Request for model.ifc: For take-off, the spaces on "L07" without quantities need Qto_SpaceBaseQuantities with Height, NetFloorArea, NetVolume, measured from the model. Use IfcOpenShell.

First a look at what the model holds.

```python
import ifcopenshell
import ifcopenshell.util.element
import ifcopenshell.util.unit

model = ifcopenshell.open("model.ifc")
print(model.schema)
for unit_type in ("LENGTHUNIT", "AREAUNIT", "VOLUMEUNIT"):
    print(unit_type, ifcopenshell.util.unit.calculate_unit_scale(model, unit_type))
storey = next(s for s in model.by_type("IfcBuildingStorey") if s.Name == "L07")
spaces = [e for e in ifcopenshell.util.element.get_decomposition(storey) if e.is_a("IfcSpace")]
for e in sorted(spaces, key=lambda e: e.id()):
    print(e.id(), e.is_a(), e.Name, list(ifcopenshell.util.element.get_psets(e, qtos_only=True)), sep=" | ")
```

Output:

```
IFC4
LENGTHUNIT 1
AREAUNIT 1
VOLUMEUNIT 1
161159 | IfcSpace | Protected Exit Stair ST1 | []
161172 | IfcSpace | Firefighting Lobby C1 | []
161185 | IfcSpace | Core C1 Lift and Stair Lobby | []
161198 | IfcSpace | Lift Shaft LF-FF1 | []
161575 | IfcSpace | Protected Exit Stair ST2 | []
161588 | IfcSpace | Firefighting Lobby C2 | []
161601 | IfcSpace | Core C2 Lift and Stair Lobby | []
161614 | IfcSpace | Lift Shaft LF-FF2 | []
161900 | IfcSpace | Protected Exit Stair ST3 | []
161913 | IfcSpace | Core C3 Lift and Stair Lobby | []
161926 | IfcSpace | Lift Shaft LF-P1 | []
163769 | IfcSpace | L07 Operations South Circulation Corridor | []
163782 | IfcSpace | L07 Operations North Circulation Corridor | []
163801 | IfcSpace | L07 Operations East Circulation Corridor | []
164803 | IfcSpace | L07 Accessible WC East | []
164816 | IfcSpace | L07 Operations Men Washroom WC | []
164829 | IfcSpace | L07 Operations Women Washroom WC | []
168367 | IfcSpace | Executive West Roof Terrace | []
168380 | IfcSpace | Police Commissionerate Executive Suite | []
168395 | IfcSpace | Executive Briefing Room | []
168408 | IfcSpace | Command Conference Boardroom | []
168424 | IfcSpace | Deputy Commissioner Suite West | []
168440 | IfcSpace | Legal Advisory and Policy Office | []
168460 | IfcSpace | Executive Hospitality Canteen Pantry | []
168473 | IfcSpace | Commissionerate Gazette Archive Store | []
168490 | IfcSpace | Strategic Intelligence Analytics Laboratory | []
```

```python
import ifcopenshell
import ifcopenshell.api.pset
import ifcopenshell.geom
import ifcopenshell.util.element
import ifcopenshell.util.shape
import ifcopenshell.util.unit

model = ifcopenshell.open("model.ifc")
unit_scale = ifcopenshell.util.unit.calculate_unit_scale(model)
area_scale = ifcopenshell.util.unit.calculate_unit_scale(model, "AREAUNIT")
volume_scale = ifcopenshell.util.unit.calculate_unit_scale(model, "VOLUMEUNIT")
settings = ifcopenshell.geom.settings()

storey = next(s for s in model.by_type("IfcBuildingStorey") if s.Name == "L07")
spaces = [e for e in ifcopenshell.util.element.get_decomposition(storey) if e.is_a("IfcSpace")]

for e in sorted(spaces, key=lambda e: e.id()):
    if ifcopenshell.util.element.get_psets(e, qtos_only=True, should_inherit=False):
        continue
    # Geometry comes back in metres, in the element's own axes.
    shape = ifcopenshell.geom.create_shape(settings, e)
    values = {
        "Height": ifcopenshell.util.shape.get_z(shape.geometry) / unit_scale,
        "NetFloorArea": ifcopenshell.util.shape.get_footprint_area(shape.geometry) / area_scale,
        "NetVolume": ifcopenshell.util.shape.get_volume(shape.geometry) / volume_scale,
    }
    qto = ifcopenshell.api.pset.add_qto(model, product=e, name="Qto_SpaceBaseQuantities")
    ifcopenshell.api.pset.edit_qto(model, qto=qto, properties=values)
    print(e.id(), {k: round(v, 3) for k, v in values.items()})

model.write("model_edited.ifc")
```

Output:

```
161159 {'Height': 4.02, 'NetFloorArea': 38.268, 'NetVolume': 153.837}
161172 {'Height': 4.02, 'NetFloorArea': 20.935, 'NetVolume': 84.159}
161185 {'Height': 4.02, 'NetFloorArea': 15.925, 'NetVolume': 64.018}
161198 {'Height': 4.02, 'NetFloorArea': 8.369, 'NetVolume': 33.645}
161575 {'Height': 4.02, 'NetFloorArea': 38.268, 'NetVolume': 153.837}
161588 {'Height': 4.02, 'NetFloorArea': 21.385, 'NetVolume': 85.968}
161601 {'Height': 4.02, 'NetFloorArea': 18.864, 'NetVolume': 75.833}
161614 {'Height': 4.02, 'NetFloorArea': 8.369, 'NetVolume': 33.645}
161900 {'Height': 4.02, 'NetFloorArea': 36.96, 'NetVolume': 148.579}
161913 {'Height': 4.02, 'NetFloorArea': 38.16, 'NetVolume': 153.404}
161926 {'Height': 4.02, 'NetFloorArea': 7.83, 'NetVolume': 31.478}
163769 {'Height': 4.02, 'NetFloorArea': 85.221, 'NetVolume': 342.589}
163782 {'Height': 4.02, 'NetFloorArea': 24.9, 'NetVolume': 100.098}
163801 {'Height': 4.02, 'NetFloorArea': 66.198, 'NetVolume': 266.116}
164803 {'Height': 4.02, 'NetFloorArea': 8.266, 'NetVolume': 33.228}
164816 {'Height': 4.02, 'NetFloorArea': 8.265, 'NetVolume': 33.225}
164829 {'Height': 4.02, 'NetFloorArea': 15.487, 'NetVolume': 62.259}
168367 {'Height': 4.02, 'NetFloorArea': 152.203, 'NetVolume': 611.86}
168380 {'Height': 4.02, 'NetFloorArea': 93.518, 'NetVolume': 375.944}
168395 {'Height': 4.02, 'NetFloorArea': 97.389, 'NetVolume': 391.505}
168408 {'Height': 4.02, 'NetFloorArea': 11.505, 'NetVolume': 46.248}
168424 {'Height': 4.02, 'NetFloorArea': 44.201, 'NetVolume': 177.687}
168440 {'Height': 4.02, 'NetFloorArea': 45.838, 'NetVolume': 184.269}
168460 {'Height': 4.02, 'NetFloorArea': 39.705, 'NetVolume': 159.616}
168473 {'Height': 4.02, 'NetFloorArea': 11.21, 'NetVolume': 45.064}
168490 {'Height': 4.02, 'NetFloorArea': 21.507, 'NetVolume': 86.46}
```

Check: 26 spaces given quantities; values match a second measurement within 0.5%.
